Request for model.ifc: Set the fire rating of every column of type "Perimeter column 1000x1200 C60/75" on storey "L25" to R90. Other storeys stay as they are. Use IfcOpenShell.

First a look at what the model holds.

```python
import ifcopenshell
import ifcopenshell.util.element

model = ifcopenshell.open("model.ifc")
print(model.schema)
storey = next(s for s in model.by_type("IfcBuildingStorey") if s.Name == "L25")
columns = [e for e in ifcopenshell.util.element.get_decomposition(storey) if e.is_a("IfcColumn")]
seen = {}
for e in columns:
    element_type = ifcopenshell.util.element.get_type(e)
    key = (element_type.Name if element_type != e and element_type else None, ifcopenshell.util.element.get_pset(e, "Pset_ColumnCommon", "FireRating"))
    seen[key] = seen.get(key, 0) + 1
for (name, value), count in sorted(seen.items(), key=str):
    print(count, "x", name, "|", value)
```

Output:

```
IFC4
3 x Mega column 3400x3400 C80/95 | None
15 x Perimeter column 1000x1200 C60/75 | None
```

```python
import ifcopenshell
import ifcopenshell.api.pset
import ifcopenshell.util.element

model = ifcopenshell.open("model.ifc")

storey = next(s for s in model.by_type("IfcBuildingStorey") if s.Name == "L25")
columns = [e for e in ifcopenshell.util.element.get_decomposition(storey) if e.is_a("IfcColumn")]

count = 0
for e in columns:
    element_type = ifcopenshell.util.element.get_type(e)
    if element_type in (None, e) or element_type.Name != "Perimeter column 1000x1200 C60/75":
        continue
    found = ifcopenshell.util.element.get_pset(e, "Pset_ColumnCommon", should_inherit=False)
    if found:
        pset = model.by_id(found["id"])
        if len(ifcopenshell.util.element.get_elements_by_pset(pset)) > 1:
            pset = ifcopenshell.api.pset.unshare_pset(model, products=[e], pset=pset)[0]
    else:
        pset = ifcopenshell.api.pset.add_pset(model, product=e, name="Pset_ColumnCommon")
    ifcopenshell.api.pset.edit_pset(model, pset=pset, properties={"FireRating": "R90"})
    count += 1

print(count, "columns updated")

model.write("model_updated.ifc")
```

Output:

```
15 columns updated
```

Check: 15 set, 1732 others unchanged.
